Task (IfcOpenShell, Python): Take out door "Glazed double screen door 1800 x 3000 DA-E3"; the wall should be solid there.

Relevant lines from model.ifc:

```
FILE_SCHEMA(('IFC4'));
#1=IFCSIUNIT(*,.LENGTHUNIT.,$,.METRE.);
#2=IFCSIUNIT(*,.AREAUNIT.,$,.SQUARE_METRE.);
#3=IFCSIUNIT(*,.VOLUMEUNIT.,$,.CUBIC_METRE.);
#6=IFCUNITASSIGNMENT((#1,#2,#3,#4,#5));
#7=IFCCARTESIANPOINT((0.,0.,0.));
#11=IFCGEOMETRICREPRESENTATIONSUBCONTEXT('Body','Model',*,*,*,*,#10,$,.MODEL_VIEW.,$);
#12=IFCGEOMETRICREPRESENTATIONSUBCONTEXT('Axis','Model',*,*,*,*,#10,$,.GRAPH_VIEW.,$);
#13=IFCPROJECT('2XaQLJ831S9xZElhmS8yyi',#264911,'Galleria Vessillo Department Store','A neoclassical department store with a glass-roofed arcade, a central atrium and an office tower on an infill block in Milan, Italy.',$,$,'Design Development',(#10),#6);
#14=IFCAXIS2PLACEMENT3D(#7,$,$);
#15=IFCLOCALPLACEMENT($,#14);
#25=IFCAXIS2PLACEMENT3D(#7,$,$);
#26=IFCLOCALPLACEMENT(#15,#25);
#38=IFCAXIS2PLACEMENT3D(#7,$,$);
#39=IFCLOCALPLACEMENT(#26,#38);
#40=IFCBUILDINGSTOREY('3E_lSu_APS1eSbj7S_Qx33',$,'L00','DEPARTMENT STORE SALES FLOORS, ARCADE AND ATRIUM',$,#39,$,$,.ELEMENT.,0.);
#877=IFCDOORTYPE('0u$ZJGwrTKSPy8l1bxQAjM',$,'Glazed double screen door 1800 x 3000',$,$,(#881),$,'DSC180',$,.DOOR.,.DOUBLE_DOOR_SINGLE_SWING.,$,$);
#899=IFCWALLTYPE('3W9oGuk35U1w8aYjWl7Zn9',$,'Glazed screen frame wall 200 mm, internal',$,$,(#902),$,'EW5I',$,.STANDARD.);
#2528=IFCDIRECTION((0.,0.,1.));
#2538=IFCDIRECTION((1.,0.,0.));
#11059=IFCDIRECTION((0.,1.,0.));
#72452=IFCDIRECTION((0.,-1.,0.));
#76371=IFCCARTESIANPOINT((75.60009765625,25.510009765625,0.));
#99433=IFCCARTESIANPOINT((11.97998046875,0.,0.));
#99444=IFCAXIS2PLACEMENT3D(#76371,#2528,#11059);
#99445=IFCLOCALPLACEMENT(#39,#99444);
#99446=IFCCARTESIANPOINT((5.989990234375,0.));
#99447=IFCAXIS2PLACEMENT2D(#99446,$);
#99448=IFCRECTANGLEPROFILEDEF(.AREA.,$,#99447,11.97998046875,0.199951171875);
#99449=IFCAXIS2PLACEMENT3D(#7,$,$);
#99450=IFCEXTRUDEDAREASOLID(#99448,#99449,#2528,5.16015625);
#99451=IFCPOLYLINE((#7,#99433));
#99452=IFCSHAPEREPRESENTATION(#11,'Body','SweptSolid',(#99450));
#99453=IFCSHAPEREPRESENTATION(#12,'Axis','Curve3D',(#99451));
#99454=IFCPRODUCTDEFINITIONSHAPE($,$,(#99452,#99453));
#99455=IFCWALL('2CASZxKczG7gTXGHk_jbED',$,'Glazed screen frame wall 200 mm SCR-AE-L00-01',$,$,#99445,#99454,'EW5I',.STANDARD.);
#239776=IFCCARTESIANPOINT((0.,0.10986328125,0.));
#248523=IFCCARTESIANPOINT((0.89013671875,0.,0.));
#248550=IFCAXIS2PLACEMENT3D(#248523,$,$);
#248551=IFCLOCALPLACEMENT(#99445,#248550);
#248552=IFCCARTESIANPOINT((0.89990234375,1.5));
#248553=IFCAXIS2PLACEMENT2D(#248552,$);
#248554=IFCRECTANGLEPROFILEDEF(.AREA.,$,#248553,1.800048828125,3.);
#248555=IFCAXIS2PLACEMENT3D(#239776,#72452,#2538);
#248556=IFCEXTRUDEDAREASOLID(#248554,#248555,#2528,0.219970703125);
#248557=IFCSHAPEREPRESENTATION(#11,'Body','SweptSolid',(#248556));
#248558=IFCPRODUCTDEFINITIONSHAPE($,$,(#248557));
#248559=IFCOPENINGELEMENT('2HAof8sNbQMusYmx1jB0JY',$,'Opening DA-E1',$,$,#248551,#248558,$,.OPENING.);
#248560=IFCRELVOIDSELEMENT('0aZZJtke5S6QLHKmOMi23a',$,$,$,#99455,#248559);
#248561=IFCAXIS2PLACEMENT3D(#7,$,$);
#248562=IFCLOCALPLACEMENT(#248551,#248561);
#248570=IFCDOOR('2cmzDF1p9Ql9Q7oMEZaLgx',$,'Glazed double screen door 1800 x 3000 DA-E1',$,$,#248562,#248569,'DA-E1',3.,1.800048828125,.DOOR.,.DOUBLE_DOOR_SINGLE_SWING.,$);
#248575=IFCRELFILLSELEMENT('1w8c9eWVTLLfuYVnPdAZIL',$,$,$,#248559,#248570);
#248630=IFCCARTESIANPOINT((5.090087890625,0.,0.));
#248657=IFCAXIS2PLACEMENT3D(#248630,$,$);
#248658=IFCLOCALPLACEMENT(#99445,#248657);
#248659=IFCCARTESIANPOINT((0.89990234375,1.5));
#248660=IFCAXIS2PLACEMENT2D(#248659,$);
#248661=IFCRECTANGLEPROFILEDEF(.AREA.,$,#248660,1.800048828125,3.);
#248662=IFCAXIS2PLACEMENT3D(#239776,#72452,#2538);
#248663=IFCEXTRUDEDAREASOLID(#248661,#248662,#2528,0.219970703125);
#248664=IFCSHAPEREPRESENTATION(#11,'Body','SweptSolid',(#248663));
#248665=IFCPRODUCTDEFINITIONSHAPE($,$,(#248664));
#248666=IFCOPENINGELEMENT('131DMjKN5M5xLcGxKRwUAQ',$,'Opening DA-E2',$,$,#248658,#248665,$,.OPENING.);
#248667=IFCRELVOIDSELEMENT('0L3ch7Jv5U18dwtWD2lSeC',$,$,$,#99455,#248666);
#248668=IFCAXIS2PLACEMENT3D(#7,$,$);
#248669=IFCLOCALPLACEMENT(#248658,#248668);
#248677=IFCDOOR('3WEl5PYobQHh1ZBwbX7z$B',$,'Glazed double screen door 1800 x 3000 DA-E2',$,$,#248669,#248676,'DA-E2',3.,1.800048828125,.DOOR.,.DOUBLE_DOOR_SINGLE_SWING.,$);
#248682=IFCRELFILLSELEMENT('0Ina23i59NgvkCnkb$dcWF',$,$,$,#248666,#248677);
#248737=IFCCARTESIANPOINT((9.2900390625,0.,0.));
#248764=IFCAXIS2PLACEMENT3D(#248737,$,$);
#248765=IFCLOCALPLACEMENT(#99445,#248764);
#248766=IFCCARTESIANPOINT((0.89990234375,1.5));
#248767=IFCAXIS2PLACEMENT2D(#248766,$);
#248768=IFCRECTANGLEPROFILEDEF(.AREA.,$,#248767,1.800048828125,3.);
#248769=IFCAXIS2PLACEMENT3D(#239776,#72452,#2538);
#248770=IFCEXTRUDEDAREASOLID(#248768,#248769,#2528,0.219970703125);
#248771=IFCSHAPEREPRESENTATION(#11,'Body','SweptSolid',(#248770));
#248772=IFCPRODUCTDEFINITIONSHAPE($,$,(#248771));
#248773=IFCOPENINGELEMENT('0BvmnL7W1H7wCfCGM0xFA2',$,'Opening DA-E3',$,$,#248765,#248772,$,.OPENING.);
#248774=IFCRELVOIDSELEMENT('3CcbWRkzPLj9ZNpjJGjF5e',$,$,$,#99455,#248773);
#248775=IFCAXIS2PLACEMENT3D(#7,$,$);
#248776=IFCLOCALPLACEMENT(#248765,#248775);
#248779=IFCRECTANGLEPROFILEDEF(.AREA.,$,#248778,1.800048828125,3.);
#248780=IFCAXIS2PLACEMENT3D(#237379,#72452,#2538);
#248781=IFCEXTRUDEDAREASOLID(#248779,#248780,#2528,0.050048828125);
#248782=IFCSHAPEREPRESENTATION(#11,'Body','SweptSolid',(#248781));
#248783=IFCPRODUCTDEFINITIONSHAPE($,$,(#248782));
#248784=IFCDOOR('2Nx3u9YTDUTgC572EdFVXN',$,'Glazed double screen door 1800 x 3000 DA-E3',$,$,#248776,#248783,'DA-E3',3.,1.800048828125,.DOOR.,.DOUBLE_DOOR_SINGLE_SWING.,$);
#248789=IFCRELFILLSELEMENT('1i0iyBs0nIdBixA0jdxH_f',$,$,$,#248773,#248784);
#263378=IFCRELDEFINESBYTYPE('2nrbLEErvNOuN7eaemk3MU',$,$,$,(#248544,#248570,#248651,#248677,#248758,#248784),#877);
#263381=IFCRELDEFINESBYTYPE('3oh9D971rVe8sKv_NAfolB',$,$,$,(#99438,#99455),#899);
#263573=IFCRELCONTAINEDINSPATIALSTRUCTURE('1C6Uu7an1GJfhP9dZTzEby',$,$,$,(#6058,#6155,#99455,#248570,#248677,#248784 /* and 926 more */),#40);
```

```python
import ifcopenshell
import ifcopenshell.api.feature
import ifcopenshell.api.root
import ifcopenshell.geom
import ifcopenshell.util.shape

model = ifcopenshell.open("model.ifc")
settings = ifcopenshell.geom.settings()


def volume(element):
    """Net volume in cubic metres, openings subtracted."""
    shape = ifcopenshell.geom.create_shape(settings, element)
    return ifcopenshell.util.shape.get_volume(shape.geometry)


door = model.by_guid("2Nx3u9YTDUTgC572EdFVXN")
opening = door.FillsVoids[0].RelatingOpeningElement
wall = opening.VoidsElements[0].RelatingBuildingElement
before = volume(wall)

ifcopenshell.api.root.remove_product(model, product=door)
ifcopenshell.api.feature.remove_feature(model, feature=opening)

after = volume(wall)

print(f"wall volume {before:.3f} -> {after:.3f} m3")

model.write("model_edited.ifc")
```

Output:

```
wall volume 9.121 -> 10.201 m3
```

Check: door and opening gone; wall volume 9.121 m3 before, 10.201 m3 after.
